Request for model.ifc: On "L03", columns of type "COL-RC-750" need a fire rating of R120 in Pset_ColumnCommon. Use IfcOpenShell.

First a look at what the model holds.

```python
import ifcopenshell
import ifcopenshell.util.element

model = ifcopenshell.open("model.ifc")
print(model.schema)
storey = next(s for s in model.by_type("IfcBuildingStorey") if s.Name == "L03")
columns = [e for e in ifcopenshell.util.element.get_decomposition(storey) if e.is_a("IfcColumn")]
seen = {}
for e in columns:
    element_type = ifcopenshell.util.element.get_type(e)
    key = (element_type.Name if element_type != e and element_type else None, ifcopenshell.util.element.get_pset(e, "Pset_ColumnCommon", "FireRating"))
    seen[key] = seen.get(key, 0) + 1
for (name, value), count in sorted(seen.items(), key=str):
    print(count, "x", name, "|", value)
```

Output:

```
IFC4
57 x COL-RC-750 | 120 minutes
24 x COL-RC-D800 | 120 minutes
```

```python
import ifcopenshell
import ifcopenshell.api.pset
import ifcopenshell.util.element

model = ifcopenshell.open("model.ifc")

storey = next(s for s in model.by_type("IfcBuildingStorey") if s.Name == "L03")
columns = [e for e in ifcopenshell.util.element.get_decomposition(storey) if e.is_a("IfcColumn")]

count = 0
for e in columns:
    element_type = ifcopenshell.util.element.get_type(e)
    if element_type in (None, e) or element_type.Name != "COL-RC-750":
        continue
    # add_pset returns the element's existing set when there is one.
    pset = ifcopenshell.api.pset.add_pset(model, product=e, name="Pset_ColumnCommon")
    ifcopenshell.api.pset.edit_pset(model, pset=pset, properties={"FireRating": "R120"})
    count += 1

print(count, "columns updated")

model.write("model-out.ifc")
```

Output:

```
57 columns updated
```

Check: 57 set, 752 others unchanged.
